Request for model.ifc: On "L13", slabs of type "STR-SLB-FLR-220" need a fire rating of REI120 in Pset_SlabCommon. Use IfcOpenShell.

First a look at what the model holds.

```python
import ifcopenshell
import ifcopenshell.util.element

model = ifcopenshell.open("model.ifc")
print(model.schema)
storey = next(s for s in model.by_type("IfcBuildingStorey") if s.Name == "L13")
slabs = [e for e in ifcopenshell.util.element.get_decomposition(storey) if e.is_a("IfcSlab")]
seen = {}
for e in slabs:
    element_type = ifcopenshell.util.element.get_type(e)
    key = (element_type.Name if element_type != e and element_type else None, ifcopenshell.util.element.get_pset(e, "Pset_SlabCommon", "FireRating"))
    seen[key] = seen.get(key, 0) + 1
for (name, value), count in sorted(seen.items(), key=str):
    print(count, "x", name, "|", value)
```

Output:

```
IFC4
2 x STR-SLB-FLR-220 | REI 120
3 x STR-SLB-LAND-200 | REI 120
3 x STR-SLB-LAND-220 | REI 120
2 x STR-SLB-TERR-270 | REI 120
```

```python
import ifcopenshell
import ifcopenshell.api.pset
import ifcopenshell.util.element

model = ifcopenshell.open("model.ifc")

storey = next(s for s in model.by_type("IfcBuildingStorey") if s.Name == "L13")
slabs = [e for e in ifcopenshell.util.element.get_decomposition(storey) if e.is_a("IfcSlab")]

count = 0
for e in slabs:
    element_type = ifcopenshell.util.element.get_type(e)
    if element_type in (None, e) or element_type.Name != "STR-SLB-FLR-220":
        continue
    # add_pset returns the element's existing set when there is one.
    pset = ifcopenshell.api.pset.add_pset(model, product=e, name="Pset_SlabCommon")
    ifcopenshell.api.pset.edit_pset(model, pset=pset, properties={"FireRating": "REI120"})
    count += 1

print(count, "slabs updated")

model.write("model_edited.ifc")
```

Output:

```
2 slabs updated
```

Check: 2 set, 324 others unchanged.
